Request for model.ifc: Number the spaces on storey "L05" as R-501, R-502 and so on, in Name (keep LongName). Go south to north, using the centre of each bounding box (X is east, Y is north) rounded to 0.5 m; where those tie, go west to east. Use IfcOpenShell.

First a look at what the model holds.

```python
import ifcopenshell
import ifcopenshell.util.element
import ifcopenshell.util.placement

model = ifcopenshell.open("model.ifc")
print(model.schema)
storey = next(s for s in model.by_type("IfcBuildingStorey") if s.Name == "L05")
spaces = [e for e in ifcopenshell.util.element.get_decomposition(storey) if e.is_a("IfcSpace")]
for e in sorted(spaces, key=lambda e: e.id()):
    origin = ifcopenshell.util.placement.get_local_placement(e.ObjectPlacement)[:3, 3]
    print(e.id(), e.Name, e.LongName, origin.round(2) + 0.0, sep=" | ")
```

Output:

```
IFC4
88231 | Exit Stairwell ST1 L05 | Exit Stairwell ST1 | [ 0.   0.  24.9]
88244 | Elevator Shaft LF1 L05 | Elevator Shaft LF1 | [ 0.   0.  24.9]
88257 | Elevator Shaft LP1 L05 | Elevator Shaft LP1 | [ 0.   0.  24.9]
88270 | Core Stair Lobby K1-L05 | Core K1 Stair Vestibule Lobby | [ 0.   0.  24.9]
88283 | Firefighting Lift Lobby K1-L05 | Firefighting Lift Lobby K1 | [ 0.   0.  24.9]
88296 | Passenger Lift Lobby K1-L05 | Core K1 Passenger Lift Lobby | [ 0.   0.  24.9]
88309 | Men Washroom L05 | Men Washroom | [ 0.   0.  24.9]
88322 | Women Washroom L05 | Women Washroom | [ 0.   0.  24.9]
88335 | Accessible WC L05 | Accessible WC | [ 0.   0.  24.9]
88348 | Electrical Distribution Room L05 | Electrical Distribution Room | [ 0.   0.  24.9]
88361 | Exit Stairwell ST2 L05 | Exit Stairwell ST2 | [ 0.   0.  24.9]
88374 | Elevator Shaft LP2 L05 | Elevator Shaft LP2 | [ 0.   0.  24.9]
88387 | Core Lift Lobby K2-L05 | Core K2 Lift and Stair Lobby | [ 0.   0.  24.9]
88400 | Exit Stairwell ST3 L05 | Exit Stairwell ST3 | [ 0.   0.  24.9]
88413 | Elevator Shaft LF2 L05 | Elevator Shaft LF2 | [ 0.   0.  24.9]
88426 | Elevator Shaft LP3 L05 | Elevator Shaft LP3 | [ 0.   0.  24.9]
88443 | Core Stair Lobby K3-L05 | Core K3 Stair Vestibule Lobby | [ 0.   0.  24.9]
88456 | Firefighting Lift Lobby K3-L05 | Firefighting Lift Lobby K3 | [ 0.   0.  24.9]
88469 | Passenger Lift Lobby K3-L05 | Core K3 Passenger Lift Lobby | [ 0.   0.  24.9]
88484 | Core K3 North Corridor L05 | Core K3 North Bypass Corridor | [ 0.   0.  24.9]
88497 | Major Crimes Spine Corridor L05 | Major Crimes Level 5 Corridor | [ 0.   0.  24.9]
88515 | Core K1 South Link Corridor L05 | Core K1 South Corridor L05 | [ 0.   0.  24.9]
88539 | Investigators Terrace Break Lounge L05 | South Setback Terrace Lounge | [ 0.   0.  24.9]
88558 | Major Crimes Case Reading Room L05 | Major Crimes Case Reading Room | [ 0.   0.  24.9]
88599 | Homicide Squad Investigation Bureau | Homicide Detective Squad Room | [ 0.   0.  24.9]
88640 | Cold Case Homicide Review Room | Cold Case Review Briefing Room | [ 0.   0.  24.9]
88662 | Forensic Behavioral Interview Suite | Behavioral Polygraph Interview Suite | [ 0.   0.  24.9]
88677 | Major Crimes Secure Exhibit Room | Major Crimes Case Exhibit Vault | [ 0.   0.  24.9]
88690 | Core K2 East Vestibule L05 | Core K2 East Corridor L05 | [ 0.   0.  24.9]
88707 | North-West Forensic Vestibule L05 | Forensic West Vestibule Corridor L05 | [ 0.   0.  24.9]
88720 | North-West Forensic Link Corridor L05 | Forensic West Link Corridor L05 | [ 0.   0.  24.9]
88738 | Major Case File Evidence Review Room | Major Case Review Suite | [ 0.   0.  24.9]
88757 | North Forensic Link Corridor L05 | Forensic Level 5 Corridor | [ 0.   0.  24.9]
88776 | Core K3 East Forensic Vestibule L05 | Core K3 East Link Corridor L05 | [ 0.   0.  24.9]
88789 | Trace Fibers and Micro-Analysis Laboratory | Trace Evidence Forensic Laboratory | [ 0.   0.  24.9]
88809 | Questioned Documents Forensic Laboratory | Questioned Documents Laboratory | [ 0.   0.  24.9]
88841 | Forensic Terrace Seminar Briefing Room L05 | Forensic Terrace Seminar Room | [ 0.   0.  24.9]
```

```python
import ifcopenshell
import ifcopenshell.geom
import ifcopenshell.util.element
import ifcopenshell.util.shape

model = ifcopenshell.open("model.ifc")
settings = ifcopenshell.geom.settings()
settings.set("use-world-coords", True)


def centre(element):
    shape = ifcopenshell.geom.create_shape(settings, element)
    return ifcopenshell.util.shape.get_bbox_centroid(shape.geometry)


storey = next(s for s in model.by_type("IfcBuildingStorey") if s.Name == "L05")
spaces = [e for e in ifcopenshell.util.element.get_decomposition(storey) if e.is_a("IfcSpace")]

# Insertion points can sit at a corner or the storey origin, so sort by the geometry (in metres).
centres = {e: centre(e) for e in spaces}
spaces.sort(key=lambda e: (round(centres[e][1] / 0.5), centres[e][0]))

for i, e in enumerate(spaces, start=1):
    number = f"R-5{i:02d}"
    e.Name = number
    print(e.id(), number)

model.write("model_v2.ifc")
```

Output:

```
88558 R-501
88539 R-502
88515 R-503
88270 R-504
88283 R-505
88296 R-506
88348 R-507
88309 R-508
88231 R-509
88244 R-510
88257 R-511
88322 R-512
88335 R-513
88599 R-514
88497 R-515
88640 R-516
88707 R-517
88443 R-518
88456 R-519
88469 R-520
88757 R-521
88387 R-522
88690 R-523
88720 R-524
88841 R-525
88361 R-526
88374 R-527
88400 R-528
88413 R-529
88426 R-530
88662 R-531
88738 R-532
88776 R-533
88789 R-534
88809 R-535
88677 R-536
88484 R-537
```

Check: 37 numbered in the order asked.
